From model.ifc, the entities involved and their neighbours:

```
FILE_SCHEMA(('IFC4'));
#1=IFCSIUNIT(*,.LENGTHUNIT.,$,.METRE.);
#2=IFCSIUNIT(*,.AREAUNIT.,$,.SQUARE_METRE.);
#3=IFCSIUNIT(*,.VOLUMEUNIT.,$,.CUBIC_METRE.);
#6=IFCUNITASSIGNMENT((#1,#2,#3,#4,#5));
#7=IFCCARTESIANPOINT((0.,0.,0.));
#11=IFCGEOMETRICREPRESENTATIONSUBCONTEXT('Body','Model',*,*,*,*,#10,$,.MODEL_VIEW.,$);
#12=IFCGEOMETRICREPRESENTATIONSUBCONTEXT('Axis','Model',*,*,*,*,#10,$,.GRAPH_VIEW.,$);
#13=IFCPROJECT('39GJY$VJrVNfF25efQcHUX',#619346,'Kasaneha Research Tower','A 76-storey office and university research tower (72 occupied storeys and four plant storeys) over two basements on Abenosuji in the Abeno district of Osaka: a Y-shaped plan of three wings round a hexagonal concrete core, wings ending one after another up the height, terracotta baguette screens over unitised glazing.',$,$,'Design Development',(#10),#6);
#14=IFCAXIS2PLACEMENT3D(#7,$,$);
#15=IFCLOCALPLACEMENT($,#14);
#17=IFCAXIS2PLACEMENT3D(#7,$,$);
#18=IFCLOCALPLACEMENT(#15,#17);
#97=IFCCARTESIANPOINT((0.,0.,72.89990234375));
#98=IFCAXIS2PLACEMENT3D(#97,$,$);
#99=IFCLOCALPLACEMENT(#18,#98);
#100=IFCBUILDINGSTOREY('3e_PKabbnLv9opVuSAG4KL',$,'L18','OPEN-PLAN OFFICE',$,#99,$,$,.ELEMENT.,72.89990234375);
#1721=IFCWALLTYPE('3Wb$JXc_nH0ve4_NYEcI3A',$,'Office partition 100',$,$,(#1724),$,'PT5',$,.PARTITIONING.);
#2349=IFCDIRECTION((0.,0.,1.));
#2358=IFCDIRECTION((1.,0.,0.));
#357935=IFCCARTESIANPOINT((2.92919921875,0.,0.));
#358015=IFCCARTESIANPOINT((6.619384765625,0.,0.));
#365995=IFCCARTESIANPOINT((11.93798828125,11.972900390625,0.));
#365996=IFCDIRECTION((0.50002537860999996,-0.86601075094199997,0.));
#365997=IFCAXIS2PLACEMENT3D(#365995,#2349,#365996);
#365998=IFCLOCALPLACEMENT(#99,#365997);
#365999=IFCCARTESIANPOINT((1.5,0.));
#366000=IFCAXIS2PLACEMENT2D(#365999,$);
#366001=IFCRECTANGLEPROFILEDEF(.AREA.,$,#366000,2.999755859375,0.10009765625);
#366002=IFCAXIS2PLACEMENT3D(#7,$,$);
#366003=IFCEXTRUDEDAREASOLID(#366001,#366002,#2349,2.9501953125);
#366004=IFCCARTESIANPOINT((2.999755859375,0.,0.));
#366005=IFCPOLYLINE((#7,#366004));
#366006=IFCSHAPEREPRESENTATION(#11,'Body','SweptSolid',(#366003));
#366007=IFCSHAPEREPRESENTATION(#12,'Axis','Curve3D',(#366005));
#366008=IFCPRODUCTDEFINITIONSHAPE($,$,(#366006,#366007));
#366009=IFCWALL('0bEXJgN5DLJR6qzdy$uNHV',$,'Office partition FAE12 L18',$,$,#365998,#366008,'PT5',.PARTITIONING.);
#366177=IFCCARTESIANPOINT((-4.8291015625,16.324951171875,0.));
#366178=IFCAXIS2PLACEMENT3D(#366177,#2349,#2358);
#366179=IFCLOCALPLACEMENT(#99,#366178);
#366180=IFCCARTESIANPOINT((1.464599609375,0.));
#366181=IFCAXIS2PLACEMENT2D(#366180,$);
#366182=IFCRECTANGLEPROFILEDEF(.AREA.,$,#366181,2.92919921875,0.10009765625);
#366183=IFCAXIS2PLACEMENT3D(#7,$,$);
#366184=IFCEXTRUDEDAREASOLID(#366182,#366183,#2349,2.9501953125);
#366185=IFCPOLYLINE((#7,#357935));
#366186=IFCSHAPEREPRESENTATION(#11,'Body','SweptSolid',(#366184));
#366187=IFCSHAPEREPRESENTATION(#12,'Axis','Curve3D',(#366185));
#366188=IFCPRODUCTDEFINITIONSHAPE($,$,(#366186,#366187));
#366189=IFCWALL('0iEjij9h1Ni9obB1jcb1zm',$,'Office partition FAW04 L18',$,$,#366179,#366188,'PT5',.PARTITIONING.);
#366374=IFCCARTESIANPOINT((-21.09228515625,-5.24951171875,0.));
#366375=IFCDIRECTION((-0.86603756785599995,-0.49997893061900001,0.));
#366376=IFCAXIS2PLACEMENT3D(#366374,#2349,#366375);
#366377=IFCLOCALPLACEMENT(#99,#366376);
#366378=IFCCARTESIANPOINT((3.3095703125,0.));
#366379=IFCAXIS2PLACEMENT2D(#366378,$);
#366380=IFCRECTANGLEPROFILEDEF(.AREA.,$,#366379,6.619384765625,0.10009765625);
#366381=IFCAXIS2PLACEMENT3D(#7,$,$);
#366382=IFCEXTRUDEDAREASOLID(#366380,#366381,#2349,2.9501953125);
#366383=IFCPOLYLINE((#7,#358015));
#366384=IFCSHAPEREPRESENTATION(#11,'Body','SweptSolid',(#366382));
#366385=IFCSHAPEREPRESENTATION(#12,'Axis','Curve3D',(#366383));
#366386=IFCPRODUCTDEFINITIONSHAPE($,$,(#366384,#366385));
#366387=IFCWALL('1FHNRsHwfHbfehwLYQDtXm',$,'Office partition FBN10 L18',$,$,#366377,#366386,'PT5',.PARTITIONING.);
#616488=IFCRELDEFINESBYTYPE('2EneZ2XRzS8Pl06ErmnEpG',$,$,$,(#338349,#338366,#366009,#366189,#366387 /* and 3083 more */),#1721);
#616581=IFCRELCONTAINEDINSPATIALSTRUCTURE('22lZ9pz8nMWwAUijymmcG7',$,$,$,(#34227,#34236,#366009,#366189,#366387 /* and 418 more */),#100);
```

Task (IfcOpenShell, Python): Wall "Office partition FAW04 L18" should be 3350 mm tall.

```python
import ifcopenshell
import ifcopenshell.geom
import ifcopenshell.util.representation
import ifcopenshell.util.shape
import ifcopenshell.util.unit

model = ifcopenshell.open("model.ifc")
unit_scale = ifcopenshell.util.unit.calculate_unit_scale(model)
settings = ifcopenshell.geom.settings()


def volume(element):
    """Net volume in cubic metres, openings subtracted."""
    shape = ifcopenshell.geom.create_shape(settings, element)
    return ifcopenshell.util.shape.get_volume(shape.geometry)


wall = model.by_guid("0iEjij9h1Ni9obB1jcb1zm")
before = volume(wall)

body = ifcopenshell.util.representation.get_representation(wall, "Model", "Body")
solid = body.Items[0]
old_height = solid.Depth
solid.Depth = 3.35 / unit_scale
after = volume(wall)

print(f"height {old_height:g} -> {solid.Depth:g}, volume {before:.3f} -> {after:.3f} m3")

model.write("model_rev.ifc")
```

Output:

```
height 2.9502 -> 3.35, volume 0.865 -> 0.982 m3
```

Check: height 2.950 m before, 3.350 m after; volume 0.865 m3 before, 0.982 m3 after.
